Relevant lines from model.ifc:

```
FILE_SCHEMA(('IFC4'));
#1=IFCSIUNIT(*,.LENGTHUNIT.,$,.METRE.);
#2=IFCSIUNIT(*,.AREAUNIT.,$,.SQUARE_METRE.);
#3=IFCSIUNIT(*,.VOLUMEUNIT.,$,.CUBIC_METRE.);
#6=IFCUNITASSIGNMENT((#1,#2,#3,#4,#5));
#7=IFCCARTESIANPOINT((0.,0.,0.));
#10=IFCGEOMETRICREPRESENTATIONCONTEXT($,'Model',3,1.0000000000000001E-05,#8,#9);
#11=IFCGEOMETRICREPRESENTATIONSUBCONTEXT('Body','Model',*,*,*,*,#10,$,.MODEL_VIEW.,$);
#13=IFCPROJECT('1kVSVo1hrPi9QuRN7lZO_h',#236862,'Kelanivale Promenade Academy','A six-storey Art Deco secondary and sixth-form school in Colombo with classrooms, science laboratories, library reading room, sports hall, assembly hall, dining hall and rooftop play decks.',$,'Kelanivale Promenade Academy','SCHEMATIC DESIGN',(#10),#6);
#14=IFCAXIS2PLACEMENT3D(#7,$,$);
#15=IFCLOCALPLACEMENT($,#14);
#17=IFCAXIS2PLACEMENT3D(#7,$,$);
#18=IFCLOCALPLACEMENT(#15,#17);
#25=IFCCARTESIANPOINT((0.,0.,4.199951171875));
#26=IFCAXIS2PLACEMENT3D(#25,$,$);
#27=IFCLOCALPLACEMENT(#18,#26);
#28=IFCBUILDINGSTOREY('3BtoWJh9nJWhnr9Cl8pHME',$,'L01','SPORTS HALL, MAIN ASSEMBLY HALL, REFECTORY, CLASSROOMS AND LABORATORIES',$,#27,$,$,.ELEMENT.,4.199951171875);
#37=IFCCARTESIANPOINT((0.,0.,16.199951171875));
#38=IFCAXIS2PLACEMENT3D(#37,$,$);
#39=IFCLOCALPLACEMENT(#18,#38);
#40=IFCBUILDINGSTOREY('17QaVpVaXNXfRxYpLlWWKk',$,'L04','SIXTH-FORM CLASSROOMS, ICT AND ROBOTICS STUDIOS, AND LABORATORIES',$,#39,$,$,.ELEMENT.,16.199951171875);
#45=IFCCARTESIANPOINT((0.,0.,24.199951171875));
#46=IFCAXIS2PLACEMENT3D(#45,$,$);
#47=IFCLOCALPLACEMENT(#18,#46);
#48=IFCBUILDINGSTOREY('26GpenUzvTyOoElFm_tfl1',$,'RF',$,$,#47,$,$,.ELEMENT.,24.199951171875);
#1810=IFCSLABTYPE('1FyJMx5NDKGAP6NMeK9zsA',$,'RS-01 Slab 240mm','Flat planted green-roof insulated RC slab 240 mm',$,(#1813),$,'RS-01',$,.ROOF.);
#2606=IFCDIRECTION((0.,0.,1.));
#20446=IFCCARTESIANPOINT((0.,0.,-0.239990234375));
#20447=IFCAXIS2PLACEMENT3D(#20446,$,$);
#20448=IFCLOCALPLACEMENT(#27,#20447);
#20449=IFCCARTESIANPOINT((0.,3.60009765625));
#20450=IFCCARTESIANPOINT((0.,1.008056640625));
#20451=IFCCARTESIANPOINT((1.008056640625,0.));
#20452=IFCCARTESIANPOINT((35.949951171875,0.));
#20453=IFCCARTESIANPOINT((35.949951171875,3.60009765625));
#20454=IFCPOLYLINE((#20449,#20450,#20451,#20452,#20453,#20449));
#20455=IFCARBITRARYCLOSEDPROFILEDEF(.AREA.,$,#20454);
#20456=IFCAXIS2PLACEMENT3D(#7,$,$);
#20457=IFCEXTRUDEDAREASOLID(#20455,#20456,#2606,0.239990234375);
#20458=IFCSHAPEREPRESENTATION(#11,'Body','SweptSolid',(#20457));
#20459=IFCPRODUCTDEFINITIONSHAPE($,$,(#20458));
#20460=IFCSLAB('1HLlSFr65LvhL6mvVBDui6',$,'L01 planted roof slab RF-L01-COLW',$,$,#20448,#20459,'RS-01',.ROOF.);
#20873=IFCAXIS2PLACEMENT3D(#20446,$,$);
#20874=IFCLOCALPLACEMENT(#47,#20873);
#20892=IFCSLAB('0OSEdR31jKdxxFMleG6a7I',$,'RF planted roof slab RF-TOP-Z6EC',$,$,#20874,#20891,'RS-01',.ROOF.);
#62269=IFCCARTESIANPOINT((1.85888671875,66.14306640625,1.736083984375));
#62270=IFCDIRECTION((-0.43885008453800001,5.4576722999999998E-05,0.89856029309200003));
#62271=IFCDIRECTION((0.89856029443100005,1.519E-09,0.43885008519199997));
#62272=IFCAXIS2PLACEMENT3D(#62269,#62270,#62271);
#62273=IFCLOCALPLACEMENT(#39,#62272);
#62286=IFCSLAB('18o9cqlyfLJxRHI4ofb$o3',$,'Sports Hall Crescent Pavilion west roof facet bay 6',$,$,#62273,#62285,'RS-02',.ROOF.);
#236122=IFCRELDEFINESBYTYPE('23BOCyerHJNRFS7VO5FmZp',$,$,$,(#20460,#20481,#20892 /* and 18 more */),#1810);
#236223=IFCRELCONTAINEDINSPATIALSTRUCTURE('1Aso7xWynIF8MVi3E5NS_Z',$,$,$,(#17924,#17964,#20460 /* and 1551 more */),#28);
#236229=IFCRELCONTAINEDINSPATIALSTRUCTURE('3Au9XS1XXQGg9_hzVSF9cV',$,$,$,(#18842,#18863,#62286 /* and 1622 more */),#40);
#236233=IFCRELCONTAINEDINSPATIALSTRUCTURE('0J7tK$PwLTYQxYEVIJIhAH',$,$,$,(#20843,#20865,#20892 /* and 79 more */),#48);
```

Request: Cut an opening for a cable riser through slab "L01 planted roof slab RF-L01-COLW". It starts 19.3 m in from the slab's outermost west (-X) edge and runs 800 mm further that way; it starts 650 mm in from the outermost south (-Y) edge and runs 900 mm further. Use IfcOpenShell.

```python
import numpy as np
import ifcopenshell
import ifcopenshell.api.feature
import ifcopenshell.api.geometry
import ifcopenshell.api.root
import ifcopenshell.geom
import ifcopenshell.util.placement
import ifcopenshell.util.representation
import ifcopenshell.util.shape
import ifcopenshell.util.unit

model = ifcopenshell.open("model.ifc")
unit_scale = ifcopenshell.util.unit.calculate_unit_scale(model)
settings = ifcopenshell.geom.settings()


def volume(element):
    """Net volume in cubic metres, openings subtracted."""
    shape = ifcopenshell.geom.create_shape(settings, element)
    return ifcopenshell.util.shape.get_volume(shape.geometry)


slab = model.by_guid("1HLlSFr65LvhL6mvVBDui6")
before = volume(slab)

# Extent in the slab's own axes, in metres. The edges named are its -X and -Y sides.
slab_shape = ifcopenshell.geom.create_shape(settings, slab)
vertices = ifcopenshell.util.shape.get_vertices(slab_shape.geometry)
x_min, y_min, bottom = vertices.min(axis=0)
top = vertices[:, 2].max()

opening = ifcopenshell.api.root.create_entity(model, ifc_class="IfcOpeningElement", name="Cable riser opening", predefined_type="OPENING")
context = ifcopenshell.util.representation.get_context(model, "Model", "Body", "MODEL_VIEW")
width, depth = 0.8, 0.9
outline = [(0.0, 0.0), (width, 0.0), (width, depth), (0.0, depth), (0.0, 0.0)]
# Overshoot both faces by 50 mm so the cut is clean.
shape = ifcopenshell.api.geometry.add_slab_representation(
    model, context=context, depth=top - bottom + 0.1, polyline=outline
)
ifcopenshell.api.geometry.assign_representation(model, product=opening, representation=shape)

matrix = ifcopenshell.util.placement.get_local_placement(slab.ObjectPlacement)
matrix[:, 3] = matrix @ np.append(np.array([x_min + 19.3, y_min + 0.65, bottom - 0.05]) / unit_scale, 1.0)
ifcopenshell.api.geometry.edit_object_placement(model, product=opening, matrix=matrix, is_si=False)
ifcopenshell.api.feature.add_feature(model, feature=opening, element=slab)

after = volume(slab)

print(f"slab volume {before:.3f} -> {after:.3f} m3")

model.write("model_rev.ifc")
```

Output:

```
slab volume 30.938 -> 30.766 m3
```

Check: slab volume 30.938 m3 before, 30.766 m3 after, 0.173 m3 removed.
